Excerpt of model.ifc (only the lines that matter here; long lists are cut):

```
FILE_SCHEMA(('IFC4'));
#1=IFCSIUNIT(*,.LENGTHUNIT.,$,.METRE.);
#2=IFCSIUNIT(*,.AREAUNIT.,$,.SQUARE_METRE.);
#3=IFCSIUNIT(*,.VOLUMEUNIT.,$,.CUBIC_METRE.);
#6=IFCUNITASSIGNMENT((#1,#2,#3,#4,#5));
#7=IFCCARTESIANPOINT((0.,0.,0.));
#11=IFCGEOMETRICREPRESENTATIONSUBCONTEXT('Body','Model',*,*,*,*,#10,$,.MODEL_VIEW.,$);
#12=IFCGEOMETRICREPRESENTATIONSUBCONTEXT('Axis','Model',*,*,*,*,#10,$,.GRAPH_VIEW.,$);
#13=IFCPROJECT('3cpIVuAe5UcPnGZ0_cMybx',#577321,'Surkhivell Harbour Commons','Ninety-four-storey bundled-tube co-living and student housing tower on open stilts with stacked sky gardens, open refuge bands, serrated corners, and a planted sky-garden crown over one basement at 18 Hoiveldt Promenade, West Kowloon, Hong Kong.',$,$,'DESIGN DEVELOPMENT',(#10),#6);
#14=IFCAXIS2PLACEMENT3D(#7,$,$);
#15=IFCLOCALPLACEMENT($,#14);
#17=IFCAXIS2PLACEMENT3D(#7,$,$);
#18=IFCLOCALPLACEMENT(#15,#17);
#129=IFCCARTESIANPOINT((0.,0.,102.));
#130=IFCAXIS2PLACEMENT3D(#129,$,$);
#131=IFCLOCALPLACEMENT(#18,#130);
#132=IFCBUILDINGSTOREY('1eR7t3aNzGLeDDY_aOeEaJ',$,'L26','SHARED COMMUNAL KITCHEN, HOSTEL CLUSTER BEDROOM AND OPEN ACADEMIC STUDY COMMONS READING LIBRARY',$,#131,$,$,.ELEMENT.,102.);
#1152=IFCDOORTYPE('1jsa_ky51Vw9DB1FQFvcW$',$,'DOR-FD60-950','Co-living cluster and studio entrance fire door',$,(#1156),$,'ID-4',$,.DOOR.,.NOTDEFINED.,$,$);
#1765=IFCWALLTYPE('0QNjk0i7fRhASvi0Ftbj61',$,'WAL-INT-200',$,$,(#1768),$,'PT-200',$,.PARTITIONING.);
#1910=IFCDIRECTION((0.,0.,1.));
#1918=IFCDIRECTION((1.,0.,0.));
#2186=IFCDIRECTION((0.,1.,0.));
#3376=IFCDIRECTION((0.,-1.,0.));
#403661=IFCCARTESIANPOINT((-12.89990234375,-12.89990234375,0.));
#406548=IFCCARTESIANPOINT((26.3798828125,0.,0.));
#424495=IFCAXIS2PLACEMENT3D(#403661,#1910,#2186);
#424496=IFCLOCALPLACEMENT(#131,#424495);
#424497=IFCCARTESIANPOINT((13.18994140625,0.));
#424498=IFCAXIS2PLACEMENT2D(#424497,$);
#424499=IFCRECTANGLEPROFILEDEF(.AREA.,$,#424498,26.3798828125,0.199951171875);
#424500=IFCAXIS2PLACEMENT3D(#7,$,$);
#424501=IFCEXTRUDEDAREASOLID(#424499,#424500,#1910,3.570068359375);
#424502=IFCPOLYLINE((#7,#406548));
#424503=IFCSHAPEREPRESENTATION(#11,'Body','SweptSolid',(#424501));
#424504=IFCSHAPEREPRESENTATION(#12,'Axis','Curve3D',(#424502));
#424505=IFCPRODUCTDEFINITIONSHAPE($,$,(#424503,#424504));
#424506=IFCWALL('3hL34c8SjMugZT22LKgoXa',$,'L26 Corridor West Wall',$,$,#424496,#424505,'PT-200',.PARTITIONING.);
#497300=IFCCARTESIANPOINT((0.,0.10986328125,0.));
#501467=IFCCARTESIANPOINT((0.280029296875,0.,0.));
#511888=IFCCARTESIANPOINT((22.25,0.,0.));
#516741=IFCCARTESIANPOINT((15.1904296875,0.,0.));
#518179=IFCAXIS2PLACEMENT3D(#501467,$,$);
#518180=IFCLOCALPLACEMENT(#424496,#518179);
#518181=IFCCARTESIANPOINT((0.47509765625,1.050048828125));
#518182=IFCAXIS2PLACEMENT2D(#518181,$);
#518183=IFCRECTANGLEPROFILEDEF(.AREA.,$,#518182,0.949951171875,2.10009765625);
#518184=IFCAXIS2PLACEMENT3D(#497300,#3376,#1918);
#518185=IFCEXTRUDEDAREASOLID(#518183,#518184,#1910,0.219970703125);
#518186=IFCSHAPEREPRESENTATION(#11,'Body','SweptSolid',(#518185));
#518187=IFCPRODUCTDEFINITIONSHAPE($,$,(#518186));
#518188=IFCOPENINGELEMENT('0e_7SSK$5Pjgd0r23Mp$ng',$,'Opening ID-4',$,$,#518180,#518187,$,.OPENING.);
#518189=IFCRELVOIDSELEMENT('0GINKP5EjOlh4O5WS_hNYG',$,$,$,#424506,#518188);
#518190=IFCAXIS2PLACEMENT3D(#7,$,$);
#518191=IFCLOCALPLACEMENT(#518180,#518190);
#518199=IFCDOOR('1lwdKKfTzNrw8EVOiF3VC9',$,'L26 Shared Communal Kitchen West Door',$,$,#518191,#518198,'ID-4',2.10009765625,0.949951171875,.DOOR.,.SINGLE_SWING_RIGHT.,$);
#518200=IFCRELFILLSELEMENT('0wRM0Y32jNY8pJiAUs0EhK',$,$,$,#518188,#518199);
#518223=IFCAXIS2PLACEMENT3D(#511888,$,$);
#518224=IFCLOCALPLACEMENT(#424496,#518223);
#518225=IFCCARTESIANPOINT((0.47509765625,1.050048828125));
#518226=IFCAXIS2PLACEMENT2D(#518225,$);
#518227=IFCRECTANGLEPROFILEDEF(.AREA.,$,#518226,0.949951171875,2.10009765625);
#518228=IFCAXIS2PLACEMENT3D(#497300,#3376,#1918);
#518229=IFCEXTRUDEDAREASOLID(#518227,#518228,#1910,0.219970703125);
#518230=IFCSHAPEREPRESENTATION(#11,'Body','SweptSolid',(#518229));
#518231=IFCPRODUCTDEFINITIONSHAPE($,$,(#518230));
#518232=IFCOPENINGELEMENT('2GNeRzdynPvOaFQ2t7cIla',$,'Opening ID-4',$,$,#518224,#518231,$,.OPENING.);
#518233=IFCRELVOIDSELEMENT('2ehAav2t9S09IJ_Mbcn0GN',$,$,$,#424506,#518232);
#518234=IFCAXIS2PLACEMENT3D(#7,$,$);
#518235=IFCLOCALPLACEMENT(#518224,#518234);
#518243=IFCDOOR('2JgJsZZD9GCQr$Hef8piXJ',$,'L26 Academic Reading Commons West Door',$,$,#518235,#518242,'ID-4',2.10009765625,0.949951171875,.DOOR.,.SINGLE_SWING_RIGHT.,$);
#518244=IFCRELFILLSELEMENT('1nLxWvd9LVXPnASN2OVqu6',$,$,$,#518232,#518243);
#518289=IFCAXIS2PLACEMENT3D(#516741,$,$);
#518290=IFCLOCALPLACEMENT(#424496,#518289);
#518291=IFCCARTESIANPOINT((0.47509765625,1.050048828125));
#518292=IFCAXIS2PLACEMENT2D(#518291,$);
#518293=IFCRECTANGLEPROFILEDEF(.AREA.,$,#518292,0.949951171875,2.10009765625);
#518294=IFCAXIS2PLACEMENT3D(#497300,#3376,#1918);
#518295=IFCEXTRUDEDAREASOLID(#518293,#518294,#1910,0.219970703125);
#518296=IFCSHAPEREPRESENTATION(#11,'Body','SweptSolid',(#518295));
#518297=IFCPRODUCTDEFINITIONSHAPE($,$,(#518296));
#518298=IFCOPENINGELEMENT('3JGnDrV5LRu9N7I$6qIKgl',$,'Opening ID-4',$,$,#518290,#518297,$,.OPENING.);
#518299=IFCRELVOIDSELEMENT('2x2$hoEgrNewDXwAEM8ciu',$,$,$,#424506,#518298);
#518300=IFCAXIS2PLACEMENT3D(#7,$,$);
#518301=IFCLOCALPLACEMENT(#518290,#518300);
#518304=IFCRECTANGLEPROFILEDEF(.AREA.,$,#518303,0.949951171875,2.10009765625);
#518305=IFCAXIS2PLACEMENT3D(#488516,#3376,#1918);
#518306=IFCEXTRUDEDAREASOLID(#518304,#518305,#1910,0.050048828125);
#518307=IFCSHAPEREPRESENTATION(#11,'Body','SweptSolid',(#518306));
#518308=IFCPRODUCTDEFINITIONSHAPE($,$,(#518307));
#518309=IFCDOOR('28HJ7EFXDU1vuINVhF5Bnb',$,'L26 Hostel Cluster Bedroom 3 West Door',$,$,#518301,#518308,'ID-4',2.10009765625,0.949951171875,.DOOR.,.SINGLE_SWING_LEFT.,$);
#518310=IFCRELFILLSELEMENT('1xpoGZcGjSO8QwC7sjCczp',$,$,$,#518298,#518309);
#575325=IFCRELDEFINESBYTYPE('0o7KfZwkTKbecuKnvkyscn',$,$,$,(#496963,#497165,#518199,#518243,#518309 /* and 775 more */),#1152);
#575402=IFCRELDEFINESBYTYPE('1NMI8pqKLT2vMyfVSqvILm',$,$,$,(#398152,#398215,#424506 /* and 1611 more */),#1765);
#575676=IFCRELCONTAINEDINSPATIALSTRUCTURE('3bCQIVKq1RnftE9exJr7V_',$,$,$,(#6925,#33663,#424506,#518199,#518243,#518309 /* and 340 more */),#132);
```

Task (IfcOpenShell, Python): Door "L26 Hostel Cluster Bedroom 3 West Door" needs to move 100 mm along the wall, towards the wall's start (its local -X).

```python
import ifcopenshell
import ifcopenshell.api.geometry
import ifcopenshell.util.placement
import ifcopenshell.util.unit

model = ifcopenshell.open("model.ifc")
unit_scale = ifcopenshell.util.unit.calculate_unit_scale(model)

door = model.by_guid("28HJ7EFXDU1vuINVhF5Bnb")
opening = door.FillsVoids[0].RelatingOpeningElement
wall = opening.VoidsElements[0].RelatingBuildingElement

wall_matrix = ifcopenshell.util.placement.get_local_placement(wall.ObjectPlacement)
shift = wall_matrix[:3, 0] * -0.1 / unit_scale
before = ifcopenshell.util.placement.get_local_placement(door.ObjectPlacement)[:3, 3].copy()

# The door is placed relative to its opening, so it follows when the opening moves.
matrix = ifcopenshell.util.placement.get_local_placement(opening.ObjectPlacement)
matrix[:3, 3] += shift
ifcopenshell.api.geometry.edit_object_placement(
    model, product=opening, matrix=matrix, is_si=False, should_transform_children=True
)

after = ifcopenshell.util.placement.get_local_placement(door.ObjectPlacement)[:3, 3]
print("door moved by", (after - before).round(3) + 0.0)

model.write("model_updated.ifc")
```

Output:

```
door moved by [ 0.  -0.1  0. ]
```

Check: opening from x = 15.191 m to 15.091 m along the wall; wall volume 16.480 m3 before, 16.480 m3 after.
